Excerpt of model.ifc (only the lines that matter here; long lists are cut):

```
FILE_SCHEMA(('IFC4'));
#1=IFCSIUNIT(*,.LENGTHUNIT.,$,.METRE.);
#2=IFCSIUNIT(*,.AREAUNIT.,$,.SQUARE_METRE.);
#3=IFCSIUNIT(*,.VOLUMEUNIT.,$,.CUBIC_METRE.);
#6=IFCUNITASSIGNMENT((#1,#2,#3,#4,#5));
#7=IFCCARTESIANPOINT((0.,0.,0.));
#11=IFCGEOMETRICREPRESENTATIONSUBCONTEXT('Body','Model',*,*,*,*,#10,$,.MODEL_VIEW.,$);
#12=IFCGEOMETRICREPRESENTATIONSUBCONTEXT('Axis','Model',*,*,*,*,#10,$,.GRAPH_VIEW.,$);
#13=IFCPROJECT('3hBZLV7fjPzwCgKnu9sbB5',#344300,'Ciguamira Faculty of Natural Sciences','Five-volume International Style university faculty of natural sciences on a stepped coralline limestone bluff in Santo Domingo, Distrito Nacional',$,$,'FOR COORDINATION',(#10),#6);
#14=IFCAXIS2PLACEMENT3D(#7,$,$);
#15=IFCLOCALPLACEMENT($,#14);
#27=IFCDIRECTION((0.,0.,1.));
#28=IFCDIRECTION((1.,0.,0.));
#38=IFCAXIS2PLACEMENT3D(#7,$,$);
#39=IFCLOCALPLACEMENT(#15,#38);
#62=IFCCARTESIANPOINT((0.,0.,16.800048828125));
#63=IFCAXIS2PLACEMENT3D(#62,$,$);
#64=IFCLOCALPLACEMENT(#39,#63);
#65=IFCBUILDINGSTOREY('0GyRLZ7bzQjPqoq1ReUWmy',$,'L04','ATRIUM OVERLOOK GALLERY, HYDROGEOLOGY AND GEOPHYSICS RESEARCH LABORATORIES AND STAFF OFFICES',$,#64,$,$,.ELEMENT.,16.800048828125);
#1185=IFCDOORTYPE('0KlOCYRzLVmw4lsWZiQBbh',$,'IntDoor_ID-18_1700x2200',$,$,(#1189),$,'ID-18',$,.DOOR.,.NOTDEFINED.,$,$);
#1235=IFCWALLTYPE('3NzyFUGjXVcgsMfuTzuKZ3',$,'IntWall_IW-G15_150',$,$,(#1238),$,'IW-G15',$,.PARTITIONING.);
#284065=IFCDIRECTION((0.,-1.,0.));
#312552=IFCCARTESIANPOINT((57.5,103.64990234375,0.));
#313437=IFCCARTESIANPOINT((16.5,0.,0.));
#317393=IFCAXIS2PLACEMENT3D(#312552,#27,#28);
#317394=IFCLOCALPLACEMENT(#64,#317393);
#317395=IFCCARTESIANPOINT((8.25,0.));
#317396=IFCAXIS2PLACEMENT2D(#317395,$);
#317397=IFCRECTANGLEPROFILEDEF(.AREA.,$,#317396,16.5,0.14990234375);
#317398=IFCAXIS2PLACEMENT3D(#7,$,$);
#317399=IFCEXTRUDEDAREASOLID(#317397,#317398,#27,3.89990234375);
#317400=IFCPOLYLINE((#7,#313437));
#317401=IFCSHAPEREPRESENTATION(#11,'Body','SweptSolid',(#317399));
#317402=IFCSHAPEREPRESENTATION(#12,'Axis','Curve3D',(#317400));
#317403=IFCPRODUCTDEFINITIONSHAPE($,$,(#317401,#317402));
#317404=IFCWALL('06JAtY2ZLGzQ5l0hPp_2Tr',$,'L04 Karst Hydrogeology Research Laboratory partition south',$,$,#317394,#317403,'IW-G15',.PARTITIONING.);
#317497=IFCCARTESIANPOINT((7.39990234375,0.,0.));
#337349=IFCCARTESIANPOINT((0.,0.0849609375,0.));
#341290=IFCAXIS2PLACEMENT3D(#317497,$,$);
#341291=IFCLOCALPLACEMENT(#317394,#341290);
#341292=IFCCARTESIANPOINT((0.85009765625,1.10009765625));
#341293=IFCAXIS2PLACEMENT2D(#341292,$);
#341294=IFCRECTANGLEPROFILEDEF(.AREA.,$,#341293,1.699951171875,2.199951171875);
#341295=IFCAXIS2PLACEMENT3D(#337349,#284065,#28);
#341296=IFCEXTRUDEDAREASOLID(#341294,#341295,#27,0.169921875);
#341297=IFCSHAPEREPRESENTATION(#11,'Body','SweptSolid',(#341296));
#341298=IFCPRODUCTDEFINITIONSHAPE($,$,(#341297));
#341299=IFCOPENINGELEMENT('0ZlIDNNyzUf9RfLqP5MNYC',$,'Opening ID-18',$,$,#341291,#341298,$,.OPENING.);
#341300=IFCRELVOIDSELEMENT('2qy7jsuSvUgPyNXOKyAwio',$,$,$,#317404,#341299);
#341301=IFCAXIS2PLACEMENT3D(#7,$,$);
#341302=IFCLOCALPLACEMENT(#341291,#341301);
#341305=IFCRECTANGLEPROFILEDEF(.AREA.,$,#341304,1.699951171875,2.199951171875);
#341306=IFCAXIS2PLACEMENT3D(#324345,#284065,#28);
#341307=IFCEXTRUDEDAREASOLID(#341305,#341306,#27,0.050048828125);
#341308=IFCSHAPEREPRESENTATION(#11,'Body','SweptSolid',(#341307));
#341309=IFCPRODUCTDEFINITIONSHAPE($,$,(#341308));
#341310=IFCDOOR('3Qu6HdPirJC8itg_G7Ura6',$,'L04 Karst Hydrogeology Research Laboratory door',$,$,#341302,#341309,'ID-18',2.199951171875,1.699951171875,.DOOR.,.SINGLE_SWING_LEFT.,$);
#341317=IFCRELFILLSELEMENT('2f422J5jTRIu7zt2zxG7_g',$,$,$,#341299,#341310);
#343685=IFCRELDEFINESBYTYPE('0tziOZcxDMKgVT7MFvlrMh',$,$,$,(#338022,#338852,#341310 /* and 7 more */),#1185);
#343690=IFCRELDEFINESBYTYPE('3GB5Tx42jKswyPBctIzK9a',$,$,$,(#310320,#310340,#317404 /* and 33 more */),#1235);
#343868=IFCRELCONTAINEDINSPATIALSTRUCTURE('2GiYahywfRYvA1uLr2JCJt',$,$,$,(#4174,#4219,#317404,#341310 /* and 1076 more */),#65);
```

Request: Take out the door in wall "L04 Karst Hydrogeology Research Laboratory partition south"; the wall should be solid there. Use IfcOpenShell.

```python
import ifcopenshell
import ifcopenshell.api.feature
import ifcopenshell.api.root
import ifcopenshell.geom
import ifcopenshell.util.shape

model = ifcopenshell.open("model.ifc")
settings = ifcopenshell.geom.settings()


def volume(element):
    """Net volume in cubic metres, openings subtracted."""
    shape = ifcopenshell.geom.create_shape(settings, element)
    return ifcopenshell.util.shape.get_volume(shape.geometry)


door = model.by_guid("3Qu6HdPirJC8itg_G7Ura6")
opening = door.FillsVoids[0].RelatingOpeningElement
wall = opening.VoidsElements[0].RelatingBuildingElement
before = volume(wall)

ifcopenshell.api.root.remove_product(model, product=door)
ifcopenshell.api.feature.remove_feature(model, feature=opening)

after = volume(wall)

print(f"wall volume {before:.3f} -> {after:.3f} m3")

model.write("model_v2.ifc")
```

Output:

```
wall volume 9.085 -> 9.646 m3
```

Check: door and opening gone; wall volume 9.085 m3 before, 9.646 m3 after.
